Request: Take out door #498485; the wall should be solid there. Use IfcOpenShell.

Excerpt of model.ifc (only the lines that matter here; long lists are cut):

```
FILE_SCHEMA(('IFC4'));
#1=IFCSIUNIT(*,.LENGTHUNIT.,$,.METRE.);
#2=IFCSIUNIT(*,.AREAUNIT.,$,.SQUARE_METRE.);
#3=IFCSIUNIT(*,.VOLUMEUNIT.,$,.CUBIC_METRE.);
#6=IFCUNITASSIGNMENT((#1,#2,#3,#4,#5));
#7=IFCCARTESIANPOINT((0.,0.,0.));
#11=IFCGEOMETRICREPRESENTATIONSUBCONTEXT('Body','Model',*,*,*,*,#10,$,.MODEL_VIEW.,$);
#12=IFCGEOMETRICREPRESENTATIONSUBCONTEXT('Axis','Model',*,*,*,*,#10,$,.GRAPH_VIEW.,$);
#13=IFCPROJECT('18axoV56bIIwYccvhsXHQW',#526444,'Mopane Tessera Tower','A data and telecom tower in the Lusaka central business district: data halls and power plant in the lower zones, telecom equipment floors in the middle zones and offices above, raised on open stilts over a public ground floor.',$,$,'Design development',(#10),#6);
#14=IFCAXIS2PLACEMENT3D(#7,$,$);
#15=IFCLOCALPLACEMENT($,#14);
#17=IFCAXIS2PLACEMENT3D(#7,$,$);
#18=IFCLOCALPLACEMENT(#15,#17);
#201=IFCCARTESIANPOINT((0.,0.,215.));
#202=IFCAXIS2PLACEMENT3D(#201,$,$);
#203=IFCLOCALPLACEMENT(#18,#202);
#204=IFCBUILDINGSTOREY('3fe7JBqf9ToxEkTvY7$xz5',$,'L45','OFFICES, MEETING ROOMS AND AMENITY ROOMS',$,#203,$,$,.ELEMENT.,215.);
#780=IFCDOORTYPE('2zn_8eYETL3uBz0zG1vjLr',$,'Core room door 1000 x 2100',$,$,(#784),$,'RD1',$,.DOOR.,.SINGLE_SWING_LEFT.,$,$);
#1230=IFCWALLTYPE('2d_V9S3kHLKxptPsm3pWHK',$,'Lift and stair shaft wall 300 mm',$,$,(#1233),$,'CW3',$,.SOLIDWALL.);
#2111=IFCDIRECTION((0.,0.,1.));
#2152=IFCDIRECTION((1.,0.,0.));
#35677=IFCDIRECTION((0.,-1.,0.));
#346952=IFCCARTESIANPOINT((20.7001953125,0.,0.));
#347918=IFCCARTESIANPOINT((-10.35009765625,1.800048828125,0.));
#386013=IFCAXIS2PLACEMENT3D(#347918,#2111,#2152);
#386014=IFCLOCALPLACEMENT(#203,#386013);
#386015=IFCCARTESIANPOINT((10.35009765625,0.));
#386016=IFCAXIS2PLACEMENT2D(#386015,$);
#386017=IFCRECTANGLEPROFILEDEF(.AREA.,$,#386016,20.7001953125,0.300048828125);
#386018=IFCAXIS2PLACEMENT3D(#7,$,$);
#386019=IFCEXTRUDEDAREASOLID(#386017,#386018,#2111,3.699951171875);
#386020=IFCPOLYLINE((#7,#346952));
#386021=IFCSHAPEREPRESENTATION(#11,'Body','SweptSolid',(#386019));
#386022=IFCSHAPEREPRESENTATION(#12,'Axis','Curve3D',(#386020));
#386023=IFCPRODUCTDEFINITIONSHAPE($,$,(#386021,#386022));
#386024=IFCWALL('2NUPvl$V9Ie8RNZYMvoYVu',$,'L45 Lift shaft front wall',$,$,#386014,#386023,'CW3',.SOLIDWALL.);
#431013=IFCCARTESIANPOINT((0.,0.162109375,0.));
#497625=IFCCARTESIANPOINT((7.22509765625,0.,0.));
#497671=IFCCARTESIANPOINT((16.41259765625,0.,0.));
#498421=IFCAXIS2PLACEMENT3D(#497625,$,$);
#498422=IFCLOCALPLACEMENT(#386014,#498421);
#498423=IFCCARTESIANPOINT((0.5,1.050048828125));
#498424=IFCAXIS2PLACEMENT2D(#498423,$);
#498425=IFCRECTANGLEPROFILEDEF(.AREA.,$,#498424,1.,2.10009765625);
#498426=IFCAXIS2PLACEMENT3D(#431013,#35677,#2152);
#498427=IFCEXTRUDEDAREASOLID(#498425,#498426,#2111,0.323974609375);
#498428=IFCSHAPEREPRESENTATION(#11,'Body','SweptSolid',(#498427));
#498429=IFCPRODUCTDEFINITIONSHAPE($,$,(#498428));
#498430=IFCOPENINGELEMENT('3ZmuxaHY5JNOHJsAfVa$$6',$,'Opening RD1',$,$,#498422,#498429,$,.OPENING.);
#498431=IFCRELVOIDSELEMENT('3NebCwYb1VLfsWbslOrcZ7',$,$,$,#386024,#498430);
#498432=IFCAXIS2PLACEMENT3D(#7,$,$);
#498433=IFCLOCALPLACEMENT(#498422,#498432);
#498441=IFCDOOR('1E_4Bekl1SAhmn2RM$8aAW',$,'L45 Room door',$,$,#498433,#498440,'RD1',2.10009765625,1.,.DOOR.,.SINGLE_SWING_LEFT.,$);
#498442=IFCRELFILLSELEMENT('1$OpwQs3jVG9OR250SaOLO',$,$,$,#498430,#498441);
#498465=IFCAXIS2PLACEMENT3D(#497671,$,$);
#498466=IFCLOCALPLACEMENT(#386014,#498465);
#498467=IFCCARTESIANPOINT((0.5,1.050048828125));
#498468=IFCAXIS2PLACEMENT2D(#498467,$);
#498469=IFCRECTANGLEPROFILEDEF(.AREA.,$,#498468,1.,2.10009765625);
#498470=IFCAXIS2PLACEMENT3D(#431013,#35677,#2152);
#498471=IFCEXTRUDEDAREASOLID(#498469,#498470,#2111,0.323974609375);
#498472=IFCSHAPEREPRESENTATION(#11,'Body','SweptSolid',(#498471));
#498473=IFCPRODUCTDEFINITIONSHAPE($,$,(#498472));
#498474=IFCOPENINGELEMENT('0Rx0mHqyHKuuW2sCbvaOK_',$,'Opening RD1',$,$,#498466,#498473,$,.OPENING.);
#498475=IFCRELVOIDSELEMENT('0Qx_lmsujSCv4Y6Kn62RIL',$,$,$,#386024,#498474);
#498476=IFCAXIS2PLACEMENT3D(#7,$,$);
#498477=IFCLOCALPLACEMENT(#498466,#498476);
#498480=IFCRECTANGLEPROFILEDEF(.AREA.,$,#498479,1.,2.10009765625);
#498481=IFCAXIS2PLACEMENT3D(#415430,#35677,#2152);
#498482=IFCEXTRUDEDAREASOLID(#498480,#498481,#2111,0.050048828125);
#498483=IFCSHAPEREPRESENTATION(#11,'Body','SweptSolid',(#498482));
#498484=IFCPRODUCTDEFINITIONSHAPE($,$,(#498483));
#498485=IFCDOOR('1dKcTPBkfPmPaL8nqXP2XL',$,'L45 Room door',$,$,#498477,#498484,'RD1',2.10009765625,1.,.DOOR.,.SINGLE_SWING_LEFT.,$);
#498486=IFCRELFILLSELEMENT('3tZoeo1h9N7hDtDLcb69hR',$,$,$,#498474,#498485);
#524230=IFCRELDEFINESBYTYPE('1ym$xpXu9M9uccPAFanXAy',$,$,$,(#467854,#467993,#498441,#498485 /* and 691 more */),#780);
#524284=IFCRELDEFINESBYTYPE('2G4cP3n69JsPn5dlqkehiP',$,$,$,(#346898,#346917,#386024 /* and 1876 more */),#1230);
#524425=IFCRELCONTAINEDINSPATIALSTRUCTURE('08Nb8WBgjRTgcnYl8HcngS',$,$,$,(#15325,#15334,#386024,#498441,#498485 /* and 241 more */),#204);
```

```python
import ifcopenshell
import ifcopenshell.api.feature
import ifcopenshell.api.root
import ifcopenshell.geom
import ifcopenshell.util.shape

model = ifcopenshell.open("model.ifc")
settings = ifcopenshell.geom.settings()


def volume(element):
    """Net volume in cubic metres, openings subtracted."""
    shape = ifcopenshell.geom.create_shape(settings, element)
    return ifcopenshell.util.shape.get_volume(shape.geometry)


door = model.by_id(498485)
opening = door.FillsVoids[0].RelatingOpeningElement
wall = opening.VoidsElements[0].RelatingBuildingElement
before = volume(wall)

ifcopenshell.api.root.remove_product(model, product=door)
ifcopenshell.api.feature.remove_feature(model, feature=opening)

after = volume(wall)

print(f"wall volume {before:.3f} -> {after:.3f} m3")

model.write("model_edited.ifc")
```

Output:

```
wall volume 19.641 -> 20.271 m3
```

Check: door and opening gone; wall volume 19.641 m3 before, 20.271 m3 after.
